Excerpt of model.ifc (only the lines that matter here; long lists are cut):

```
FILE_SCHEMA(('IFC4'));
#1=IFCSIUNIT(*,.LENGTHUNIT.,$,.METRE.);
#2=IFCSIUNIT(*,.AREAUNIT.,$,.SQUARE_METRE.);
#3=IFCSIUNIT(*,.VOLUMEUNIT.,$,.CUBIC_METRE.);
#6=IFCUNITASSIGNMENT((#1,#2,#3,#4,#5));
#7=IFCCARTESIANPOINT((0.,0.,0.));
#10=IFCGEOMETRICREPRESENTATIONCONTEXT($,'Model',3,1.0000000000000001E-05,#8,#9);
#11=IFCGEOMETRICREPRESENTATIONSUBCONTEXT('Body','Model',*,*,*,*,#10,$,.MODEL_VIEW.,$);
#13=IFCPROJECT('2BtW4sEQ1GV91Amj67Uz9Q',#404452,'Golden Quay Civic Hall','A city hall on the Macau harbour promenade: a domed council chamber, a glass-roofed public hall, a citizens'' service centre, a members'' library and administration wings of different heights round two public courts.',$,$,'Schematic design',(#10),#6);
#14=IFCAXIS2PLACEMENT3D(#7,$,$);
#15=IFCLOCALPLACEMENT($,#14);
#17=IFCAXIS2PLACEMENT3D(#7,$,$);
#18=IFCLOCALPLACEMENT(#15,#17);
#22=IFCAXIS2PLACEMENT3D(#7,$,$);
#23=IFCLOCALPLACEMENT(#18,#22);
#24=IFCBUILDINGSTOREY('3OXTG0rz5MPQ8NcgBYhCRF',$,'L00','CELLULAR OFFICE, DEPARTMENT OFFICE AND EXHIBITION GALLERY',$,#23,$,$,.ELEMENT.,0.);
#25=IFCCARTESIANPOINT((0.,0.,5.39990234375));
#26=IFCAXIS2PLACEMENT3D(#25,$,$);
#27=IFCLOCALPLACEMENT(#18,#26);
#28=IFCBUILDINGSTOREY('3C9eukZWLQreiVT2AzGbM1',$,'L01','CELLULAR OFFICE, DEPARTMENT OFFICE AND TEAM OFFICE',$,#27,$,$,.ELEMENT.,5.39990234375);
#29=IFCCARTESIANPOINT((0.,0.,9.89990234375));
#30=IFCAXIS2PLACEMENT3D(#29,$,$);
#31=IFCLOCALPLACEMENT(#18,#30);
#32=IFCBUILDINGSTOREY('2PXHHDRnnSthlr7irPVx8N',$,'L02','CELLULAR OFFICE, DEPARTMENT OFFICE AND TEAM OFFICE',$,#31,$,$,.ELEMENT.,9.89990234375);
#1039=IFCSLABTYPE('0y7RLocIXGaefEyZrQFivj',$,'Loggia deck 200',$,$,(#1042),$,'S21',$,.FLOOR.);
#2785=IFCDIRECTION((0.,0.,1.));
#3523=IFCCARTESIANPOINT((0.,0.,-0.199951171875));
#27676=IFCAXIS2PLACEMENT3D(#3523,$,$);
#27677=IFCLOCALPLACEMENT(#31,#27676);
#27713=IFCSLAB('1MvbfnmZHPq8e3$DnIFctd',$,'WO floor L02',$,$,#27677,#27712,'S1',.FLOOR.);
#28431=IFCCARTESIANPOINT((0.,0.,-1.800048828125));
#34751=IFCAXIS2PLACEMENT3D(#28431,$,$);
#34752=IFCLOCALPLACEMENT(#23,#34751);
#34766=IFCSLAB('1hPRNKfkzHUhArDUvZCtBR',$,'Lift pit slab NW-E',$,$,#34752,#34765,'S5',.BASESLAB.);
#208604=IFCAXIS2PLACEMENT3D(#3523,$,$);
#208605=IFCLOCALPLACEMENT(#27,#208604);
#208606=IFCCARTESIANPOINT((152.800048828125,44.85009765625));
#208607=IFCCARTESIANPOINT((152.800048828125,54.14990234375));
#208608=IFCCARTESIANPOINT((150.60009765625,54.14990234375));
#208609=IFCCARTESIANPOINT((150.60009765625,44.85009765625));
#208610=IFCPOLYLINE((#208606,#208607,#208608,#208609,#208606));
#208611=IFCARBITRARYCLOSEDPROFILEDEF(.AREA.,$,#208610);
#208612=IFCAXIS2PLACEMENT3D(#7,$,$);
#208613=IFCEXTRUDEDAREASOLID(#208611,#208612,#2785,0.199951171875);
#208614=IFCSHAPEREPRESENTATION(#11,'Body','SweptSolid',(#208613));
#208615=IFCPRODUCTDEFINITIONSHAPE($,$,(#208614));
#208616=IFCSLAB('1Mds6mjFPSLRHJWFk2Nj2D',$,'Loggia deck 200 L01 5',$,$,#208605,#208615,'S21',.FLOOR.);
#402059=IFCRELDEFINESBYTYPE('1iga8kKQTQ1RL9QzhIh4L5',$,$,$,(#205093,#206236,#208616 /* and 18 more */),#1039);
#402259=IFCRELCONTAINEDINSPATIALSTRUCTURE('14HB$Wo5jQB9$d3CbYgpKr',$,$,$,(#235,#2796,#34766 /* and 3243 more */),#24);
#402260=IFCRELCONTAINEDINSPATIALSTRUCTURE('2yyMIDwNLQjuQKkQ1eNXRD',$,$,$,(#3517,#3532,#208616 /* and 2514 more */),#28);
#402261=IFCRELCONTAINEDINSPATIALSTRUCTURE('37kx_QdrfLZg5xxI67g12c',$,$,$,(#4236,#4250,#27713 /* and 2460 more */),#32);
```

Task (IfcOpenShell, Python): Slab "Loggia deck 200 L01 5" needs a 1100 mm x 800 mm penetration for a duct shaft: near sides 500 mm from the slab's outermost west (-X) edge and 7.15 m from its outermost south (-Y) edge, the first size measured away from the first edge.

```python
import numpy as np
import ifcopenshell
import ifcopenshell.api.feature
import ifcopenshell.api.geometry
import ifcopenshell.api.root
import ifcopenshell.geom
import ifcopenshell.util.placement
import ifcopenshell.util.representation
import ifcopenshell.util.shape
import ifcopenshell.util.unit

model = ifcopenshell.open("model.ifc")
unit_scale = ifcopenshell.util.unit.calculate_unit_scale(model)
settings = ifcopenshell.geom.settings()


def volume(element):
    """Net volume in cubic metres, openings subtracted."""
    shape = ifcopenshell.geom.create_shape(settings, element)
    return ifcopenshell.util.shape.get_volume(shape.geometry)


slab = model.by_id(208616)
before = volume(slab)

# Extent in the slab's own axes, in metres. The edges named are its -X and -Y sides.
slab_shape = ifcopenshell.geom.create_shape(settings, slab)
vertices = ifcopenshell.util.shape.get_vertices(slab_shape.geometry)
x_min, y_min, bottom = vertices.min(axis=0)
top = vertices[:, 2].max()

opening = ifcopenshell.api.root.create_entity(model, ifc_class="IfcOpeningElement", name="Duct shaft opening", predefined_type="OPENING")
context = ifcopenshell.util.representation.get_context(model, "Model", "Body", "MODEL_VIEW")
width, depth = 1.1, 0.8
outline = [(0.0, 0.0), (width, 0.0), (width, depth), (0.0, depth), (0.0, 0.0)]
# Overshoot both faces by 50 mm so the cut is clean.
shape = ifcopenshell.api.geometry.add_slab_representation(
    model, context=context, depth=top - bottom + 0.1, polyline=outline
)
ifcopenshell.api.geometry.assign_representation(model, product=opening, representation=shape)

matrix = ifcopenshell.util.placement.get_local_placement(slab.ObjectPlacement)
matrix[:, 3] = matrix @ np.append(np.array([x_min + 0.5, y_min + 7.15, bottom - 0.05]) / unit_scale, 1.0)
ifcopenshell.api.geometry.edit_object_placement(model, product=opening, matrix=matrix, is_si=False)
ifcopenshell.api.feature.add_feature(model, feature=opening, element=slab)

after = volume(slab)

print(f"slab volume {before:.3f} -> {after:.3f} m3")

model.write("model_edited.ifc")
```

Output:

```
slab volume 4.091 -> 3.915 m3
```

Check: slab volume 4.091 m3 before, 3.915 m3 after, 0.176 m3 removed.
